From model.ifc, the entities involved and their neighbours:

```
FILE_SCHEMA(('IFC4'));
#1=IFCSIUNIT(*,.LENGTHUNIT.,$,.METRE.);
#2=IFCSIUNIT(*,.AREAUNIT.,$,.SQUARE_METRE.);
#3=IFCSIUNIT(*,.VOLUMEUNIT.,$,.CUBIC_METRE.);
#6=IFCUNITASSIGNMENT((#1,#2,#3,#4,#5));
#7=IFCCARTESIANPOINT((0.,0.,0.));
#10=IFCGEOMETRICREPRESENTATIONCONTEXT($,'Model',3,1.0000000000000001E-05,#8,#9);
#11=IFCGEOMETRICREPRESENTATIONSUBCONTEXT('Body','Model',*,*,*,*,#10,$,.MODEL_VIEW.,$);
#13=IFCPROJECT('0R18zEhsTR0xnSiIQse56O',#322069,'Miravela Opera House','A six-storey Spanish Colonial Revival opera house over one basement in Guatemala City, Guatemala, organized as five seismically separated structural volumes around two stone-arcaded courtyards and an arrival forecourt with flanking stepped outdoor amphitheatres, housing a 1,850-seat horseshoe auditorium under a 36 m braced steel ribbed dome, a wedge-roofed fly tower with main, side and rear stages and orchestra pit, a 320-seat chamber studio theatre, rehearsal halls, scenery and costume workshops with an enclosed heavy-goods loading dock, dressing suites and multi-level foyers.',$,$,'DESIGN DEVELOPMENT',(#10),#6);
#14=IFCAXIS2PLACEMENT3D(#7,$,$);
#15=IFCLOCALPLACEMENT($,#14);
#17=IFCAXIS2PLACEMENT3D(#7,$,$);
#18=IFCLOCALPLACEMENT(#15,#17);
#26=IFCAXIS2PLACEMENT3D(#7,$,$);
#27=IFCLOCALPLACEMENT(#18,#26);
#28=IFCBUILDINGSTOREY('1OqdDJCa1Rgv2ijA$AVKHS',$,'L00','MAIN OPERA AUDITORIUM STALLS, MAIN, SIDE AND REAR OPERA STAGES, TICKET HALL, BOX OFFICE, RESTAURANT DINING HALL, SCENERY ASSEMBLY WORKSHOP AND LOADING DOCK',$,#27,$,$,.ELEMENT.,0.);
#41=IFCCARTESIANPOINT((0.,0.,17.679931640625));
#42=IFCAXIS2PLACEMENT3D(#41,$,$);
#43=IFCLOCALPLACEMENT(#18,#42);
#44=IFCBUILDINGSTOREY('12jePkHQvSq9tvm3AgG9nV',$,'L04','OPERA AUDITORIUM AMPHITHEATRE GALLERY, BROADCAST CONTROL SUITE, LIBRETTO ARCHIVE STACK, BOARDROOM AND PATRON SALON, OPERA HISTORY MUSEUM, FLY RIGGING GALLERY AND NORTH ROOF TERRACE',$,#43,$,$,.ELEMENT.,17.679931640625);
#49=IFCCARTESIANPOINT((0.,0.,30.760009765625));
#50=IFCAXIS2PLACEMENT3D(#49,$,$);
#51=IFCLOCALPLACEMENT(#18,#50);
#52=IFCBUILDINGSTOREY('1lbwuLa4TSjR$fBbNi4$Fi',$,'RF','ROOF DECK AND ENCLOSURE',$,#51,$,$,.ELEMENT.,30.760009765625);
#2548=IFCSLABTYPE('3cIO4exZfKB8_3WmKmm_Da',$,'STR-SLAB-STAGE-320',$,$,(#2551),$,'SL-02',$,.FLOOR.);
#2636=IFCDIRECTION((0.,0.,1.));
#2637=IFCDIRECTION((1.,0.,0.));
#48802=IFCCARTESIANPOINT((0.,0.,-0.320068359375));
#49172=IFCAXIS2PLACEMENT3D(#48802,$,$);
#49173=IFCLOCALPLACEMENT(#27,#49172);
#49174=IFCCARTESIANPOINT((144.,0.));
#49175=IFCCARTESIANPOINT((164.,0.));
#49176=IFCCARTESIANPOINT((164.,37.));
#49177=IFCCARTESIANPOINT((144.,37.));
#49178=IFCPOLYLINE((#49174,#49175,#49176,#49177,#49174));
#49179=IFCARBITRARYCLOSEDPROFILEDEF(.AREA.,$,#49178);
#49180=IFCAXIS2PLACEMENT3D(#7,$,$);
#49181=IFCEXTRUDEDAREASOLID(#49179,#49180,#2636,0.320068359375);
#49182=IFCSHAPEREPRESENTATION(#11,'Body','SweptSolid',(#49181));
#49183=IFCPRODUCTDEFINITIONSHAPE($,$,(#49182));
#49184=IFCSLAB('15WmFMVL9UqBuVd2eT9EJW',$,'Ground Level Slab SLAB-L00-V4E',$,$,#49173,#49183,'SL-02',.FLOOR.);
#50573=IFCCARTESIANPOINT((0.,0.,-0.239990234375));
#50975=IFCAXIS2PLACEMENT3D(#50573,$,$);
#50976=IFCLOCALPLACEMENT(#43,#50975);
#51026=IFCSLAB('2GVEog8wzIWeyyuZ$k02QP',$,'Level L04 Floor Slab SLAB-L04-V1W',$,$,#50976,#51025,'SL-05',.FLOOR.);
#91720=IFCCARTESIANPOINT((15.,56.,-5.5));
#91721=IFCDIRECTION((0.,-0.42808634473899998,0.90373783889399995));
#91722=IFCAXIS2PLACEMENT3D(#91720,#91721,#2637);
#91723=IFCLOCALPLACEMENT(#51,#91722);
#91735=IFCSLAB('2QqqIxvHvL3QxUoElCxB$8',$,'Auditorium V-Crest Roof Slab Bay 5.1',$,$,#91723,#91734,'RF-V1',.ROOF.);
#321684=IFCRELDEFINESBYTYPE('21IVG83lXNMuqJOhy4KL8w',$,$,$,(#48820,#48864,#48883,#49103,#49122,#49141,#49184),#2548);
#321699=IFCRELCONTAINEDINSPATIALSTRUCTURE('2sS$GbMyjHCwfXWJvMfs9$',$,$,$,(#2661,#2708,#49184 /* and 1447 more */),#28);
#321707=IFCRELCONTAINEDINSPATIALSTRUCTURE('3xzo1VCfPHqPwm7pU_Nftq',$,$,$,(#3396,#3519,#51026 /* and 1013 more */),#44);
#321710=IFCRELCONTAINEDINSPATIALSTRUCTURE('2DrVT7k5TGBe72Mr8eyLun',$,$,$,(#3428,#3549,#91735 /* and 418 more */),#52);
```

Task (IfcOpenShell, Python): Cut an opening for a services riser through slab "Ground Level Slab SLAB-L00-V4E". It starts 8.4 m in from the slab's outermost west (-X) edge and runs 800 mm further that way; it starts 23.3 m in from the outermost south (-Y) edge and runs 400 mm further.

```python
import numpy as np
import ifcopenshell
import ifcopenshell.api.feature
import ifcopenshell.api.geometry
import ifcopenshell.api.root
import ifcopenshell.geom
import ifcopenshell.util.placement
import ifcopenshell.util.representation
import ifcopenshell.util.shape
import ifcopenshell.util.unit

model = ifcopenshell.open("model.ifc")
unit_scale = ifcopenshell.util.unit.calculate_unit_scale(model)
settings = ifcopenshell.geom.settings()


def volume(element):
    """Net volume in cubic metres, openings subtracted."""
    shape = ifcopenshell.geom.create_shape(settings, element)
    return ifcopenshell.util.shape.get_volume(shape.geometry)


slab = model.by_guid("15WmFMVL9UqBuVd2eT9EJW")
before = volume(slab)

# Extent in the slab's own axes, in metres. The edges named are its -X and -Y sides.
slab_shape = ifcopenshell.geom.create_shape(settings, slab)
vertices = ifcopenshell.util.shape.get_vertices(slab_shape.geometry)
x_min, y_min, bottom = vertices.min(axis=0)
top = vertices[:, 2].max()

opening = ifcopenshell.api.root.create_entity(model, ifc_class="IfcOpeningElement", name="Services riser opening", predefined_type="OPENING")
context = ifcopenshell.util.representation.get_context(model, "Model", "Body", "MODEL_VIEW")
width, depth = 0.8, 0.4
outline = [(0.0, 0.0), (width, 0.0), (width, depth), (0.0, depth), (0.0, 0.0)]
# Overshoot both faces by 50 mm so the cut is clean.
shape = ifcopenshell.api.geometry.add_slab_representation(
    model, context=context, depth=top - bottom + 0.1, polyline=outline
)
ifcopenshell.api.geometry.assign_representation(model, product=opening, representation=shape)

matrix = ifcopenshell.util.placement.get_local_placement(slab.ObjectPlacement)
matrix[:, 3] = matrix @ np.append(np.array([x_min + 8.4, y_min + 23.3, bottom - 0.05]) / unit_scale, 1.0)
ifcopenshell.api.geometry.edit_object_placement(model, product=opening, matrix=matrix, is_si=False)
ifcopenshell.api.feature.add_feature(model, feature=opening, element=slab)

after = volume(slab)

print(f"slab volume {before:.3f} -> {after:.3f} m3")

model.write("model_v2.ifc")
```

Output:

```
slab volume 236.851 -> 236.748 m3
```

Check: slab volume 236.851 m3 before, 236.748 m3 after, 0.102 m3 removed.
